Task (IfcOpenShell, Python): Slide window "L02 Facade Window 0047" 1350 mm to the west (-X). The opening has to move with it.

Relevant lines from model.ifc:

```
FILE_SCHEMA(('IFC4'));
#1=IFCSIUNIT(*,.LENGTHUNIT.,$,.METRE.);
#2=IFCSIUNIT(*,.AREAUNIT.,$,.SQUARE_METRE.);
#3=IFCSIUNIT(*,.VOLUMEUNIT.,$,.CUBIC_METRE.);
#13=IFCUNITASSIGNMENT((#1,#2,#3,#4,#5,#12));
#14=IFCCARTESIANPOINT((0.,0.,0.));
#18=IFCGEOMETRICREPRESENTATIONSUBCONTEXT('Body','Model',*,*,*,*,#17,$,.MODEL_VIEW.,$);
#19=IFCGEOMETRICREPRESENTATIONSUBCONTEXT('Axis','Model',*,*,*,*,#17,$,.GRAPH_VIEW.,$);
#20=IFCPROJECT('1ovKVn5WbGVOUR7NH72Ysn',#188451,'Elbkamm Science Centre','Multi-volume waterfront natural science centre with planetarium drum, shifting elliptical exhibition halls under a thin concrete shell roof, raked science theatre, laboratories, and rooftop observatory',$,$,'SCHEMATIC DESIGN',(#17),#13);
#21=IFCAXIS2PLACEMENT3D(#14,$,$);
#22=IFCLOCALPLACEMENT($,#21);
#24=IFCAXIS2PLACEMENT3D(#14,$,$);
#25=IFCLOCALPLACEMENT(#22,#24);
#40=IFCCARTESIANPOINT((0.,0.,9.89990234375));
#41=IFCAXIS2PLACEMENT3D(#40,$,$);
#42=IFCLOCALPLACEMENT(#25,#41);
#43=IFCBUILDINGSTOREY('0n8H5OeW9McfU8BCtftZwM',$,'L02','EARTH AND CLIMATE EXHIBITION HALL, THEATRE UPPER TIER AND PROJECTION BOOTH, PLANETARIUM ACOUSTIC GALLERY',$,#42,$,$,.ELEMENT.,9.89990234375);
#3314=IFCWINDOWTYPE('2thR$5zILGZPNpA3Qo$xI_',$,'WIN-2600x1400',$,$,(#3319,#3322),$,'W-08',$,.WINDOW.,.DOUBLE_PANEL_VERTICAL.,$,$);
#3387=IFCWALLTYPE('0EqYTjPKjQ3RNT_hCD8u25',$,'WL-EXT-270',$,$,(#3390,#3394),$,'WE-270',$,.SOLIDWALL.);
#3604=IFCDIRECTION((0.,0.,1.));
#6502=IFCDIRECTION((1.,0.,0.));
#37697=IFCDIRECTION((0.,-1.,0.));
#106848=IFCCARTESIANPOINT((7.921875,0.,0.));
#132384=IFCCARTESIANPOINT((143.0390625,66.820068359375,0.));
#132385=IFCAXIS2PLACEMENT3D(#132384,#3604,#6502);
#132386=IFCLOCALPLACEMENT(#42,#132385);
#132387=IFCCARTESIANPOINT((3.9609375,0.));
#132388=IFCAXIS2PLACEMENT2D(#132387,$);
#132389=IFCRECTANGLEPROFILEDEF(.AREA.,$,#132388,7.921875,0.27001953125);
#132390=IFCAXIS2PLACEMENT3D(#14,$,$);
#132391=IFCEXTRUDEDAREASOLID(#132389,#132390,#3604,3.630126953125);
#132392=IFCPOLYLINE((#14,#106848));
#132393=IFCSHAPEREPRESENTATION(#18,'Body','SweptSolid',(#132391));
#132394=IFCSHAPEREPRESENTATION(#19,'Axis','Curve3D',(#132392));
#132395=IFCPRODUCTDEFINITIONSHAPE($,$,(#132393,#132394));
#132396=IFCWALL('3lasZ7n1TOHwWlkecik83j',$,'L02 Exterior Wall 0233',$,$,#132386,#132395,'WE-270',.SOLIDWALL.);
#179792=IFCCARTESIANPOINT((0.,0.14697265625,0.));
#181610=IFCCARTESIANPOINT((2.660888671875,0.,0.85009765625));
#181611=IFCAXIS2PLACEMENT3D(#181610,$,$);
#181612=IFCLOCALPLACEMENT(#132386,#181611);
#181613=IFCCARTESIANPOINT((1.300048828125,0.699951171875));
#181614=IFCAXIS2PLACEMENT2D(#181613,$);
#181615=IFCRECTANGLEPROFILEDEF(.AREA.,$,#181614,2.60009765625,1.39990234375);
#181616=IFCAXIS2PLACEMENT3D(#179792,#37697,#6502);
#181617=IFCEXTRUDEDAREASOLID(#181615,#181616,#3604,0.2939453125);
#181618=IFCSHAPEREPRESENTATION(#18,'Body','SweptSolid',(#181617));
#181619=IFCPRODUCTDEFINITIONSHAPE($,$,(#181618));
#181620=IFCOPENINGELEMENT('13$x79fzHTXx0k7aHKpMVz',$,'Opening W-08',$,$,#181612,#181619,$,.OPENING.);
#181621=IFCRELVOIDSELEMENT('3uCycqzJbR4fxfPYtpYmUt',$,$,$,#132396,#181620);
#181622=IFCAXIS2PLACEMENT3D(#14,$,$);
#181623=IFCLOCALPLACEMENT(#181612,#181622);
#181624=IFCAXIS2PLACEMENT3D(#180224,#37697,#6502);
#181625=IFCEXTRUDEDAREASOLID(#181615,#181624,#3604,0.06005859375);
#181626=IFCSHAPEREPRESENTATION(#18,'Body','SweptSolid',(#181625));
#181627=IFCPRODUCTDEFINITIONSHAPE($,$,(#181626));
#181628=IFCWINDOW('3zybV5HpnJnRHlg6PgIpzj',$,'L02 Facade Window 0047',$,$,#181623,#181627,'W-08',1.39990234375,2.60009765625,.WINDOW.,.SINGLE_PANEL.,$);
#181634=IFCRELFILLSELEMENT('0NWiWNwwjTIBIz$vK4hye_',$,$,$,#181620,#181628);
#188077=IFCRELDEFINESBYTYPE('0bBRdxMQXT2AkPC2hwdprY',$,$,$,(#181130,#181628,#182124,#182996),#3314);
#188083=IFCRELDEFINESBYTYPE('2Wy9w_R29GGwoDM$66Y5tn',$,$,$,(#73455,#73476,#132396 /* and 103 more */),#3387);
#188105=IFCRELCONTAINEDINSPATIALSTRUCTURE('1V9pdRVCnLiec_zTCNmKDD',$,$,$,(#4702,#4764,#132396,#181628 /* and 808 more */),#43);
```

```python
import ifcopenshell
import ifcopenshell.api.geometry
import ifcopenshell.util.placement
import ifcopenshell.util.unit

model = ifcopenshell.open("model.ifc")
unit_scale = ifcopenshell.util.unit.calculate_unit_scale(model)

window = model.by_guid("3zybV5HpnJnRHlg6PgIpzj")
opening = window.FillsVoids[0].RelatingOpeningElement
wall = opening.VoidsElements[0].RelatingBuildingElement

wall_matrix = ifcopenshell.util.placement.get_local_placement(wall.ObjectPlacement)
shift = wall_matrix[:3, 0] * -1.35 / unit_scale
before = ifcopenshell.util.placement.get_local_placement(window.ObjectPlacement)[:3, 3].copy()

# The window is placed relative to its opening, so it follows when the opening moves.
matrix = ifcopenshell.util.placement.get_local_placement(opening.ObjectPlacement)
matrix[:3, 3] += shift
ifcopenshell.api.geometry.edit_object_placement(
    model, product=opening, matrix=matrix, is_si=False, should_transform_children=True
)

after = ifcopenshell.util.placement.get_local_placement(window.ObjectPlacement)[:3, 3]
print("window moved by", (after - before).round(3) + 0.0)

model.write("model_edited.ifc")
```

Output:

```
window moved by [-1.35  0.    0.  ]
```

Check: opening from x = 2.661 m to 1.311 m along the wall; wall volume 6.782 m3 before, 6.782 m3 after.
